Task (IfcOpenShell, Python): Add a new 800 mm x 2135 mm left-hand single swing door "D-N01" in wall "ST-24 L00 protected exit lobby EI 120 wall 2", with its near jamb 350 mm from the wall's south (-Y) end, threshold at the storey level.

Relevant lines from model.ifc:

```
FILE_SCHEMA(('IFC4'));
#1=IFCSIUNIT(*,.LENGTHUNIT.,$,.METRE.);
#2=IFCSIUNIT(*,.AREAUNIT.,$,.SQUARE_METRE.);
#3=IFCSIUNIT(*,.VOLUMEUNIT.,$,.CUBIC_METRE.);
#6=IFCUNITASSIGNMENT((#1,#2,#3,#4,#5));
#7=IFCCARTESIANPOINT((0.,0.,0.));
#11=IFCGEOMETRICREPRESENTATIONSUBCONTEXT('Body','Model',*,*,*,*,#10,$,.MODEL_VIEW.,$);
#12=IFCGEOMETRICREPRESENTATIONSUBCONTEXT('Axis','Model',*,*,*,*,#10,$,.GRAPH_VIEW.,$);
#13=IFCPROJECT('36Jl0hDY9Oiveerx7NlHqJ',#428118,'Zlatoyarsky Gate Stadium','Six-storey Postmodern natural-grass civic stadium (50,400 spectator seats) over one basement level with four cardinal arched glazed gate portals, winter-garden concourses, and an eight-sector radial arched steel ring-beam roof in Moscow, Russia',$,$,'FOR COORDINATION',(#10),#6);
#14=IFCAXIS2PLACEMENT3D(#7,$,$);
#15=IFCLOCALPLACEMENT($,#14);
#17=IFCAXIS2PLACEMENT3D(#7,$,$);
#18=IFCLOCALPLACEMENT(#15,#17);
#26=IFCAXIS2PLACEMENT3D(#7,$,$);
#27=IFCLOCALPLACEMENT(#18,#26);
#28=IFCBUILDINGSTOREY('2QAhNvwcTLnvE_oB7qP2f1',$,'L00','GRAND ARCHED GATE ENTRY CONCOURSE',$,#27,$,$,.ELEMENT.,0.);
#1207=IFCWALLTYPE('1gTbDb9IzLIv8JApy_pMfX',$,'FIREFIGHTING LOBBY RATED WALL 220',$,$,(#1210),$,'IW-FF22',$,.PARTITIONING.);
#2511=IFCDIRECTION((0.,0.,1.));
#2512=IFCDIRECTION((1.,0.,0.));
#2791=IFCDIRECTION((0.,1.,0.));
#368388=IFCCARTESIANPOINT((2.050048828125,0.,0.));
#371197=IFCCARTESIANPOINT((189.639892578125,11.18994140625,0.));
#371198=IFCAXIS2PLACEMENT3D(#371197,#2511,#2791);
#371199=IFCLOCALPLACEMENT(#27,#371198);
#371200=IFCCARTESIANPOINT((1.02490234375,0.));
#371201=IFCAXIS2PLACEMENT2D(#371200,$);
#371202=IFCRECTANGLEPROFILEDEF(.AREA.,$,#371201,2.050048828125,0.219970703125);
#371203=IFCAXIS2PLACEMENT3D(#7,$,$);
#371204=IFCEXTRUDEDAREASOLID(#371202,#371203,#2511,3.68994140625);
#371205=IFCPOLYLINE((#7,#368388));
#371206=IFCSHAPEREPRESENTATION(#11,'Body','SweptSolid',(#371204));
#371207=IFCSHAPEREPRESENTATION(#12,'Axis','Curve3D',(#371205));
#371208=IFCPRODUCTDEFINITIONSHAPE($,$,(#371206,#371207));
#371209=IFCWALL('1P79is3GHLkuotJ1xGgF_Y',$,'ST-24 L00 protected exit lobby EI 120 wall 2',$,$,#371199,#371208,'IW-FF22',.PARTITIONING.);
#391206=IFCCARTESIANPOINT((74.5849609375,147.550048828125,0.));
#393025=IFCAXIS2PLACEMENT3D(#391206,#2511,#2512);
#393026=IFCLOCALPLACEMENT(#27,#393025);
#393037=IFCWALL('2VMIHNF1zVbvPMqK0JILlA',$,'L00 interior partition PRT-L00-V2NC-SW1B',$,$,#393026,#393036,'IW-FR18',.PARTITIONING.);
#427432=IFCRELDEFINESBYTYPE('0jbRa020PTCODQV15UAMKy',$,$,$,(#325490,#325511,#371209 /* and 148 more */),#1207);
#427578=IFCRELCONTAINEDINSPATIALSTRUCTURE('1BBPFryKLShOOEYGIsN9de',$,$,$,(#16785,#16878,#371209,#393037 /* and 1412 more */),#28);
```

```python
import numpy as np
import ifcopenshell
import ifcopenshell.api.feature
import ifcopenshell.api.geometry
import ifcopenshell.api.root
import ifcopenshell.api.spatial
import ifcopenshell.geom
import ifcopenshell.util.element
import ifcopenshell.util.placement
import ifcopenshell.util.representation
import ifcopenshell.util.shape
import ifcopenshell.util.unit

model = ifcopenshell.open("model.ifc")
unit_scale = ifcopenshell.util.unit.calculate_unit_scale(model)
settings = ifcopenshell.geom.settings()


def volume(element):
    """Net volume in cubic metres, openings subtracted."""
    shape = ifcopenshell.geom.create_shape(settings, element)
    return ifcopenshell.util.shape.get_volume(shape.geometry)


wall = model.by_id(371209)
storey = ifcopenshell.util.element.get_container(wall, ifc_class="IfcBuildingStorey")
context = ifcopenshell.util.representation.get_context(model, "Model", "Body", "MODEL_VIEW")
before = volume(wall)

width, height, from_end, sill = 0.8, 2.135, 0.35, 0.0  # metres

# The wall runs along its own X axis, and the end named is its -X end.
wall_shape = ifcopenshell.geom.create_shape(settings, wall)
x, y, z = ifcopenshell.util.shape.get_vertices(wall_shape.geometry).T
start = x.min() + from_end
face, thickness = float(y.min()), float(y.max() - y.min())
wall_matrix = ifcopenshell.util.placement.get_local_placement(wall.ObjectPlacement)
level = ifcopenshell.util.placement.get_local_placement(storey.ObjectPlacement)[2, 3]


def in_wall(x, y):
    """Placement at x, y metres in the wall's axes, at sill height."""
    matrix = wall_matrix.copy()
    matrix[:, 3] = wall_matrix @ np.array([x / unit_scale, y / unit_scale, 0.0, 1.0])
    matrix[2, 3] = level + sill / unit_scale
    return matrix


# Opening: a box that overshoots both wall faces by 50 mm.
opening = ifcopenshell.api.root.create_entity(model, ifc_class="IfcOpeningElement", predefined_type="OPENING")
box = ifcopenshell.api.geometry.add_wall_representation(
    model, context=context, length=width, height=height, thickness=thickness + 0.1
)
ifcopenshell.api.geometry.assign_representation(model, product=opening, representation=box)
ifcopenshell.api.geometry.edit_object_placement(model, product=opening, matrix=in_wall(start, face - 0.05), is_si=False)
ifcopenshell.api.feature.add_feature(model, feature=opening, element=wall)

door = ifcopenshell.api.root.create_entity(model, ifc_class="IfcDoor", name="D-N01", predefined_type="DOOR")
door.OverallWidth, door.OverallHeight = width / unit_scale, height / unit_scale
door.OperationType = "SINGLE_SWING_LEFT"
body = ifcopenshell.api.geometry.add_door_representation(
    model,
    context=context,
    overall_width=door.OverallWidth,
    overall_height=door.OverallHeight,
    operation_type="SINGLE_SWING_LEFT",
    lining_properties={"LiningDepth": thickness / unit_scale, "ThresholdDepth": thickness / unit_scale},
)
ifcopenshell.api.geometry.assign_representation(model, product=door, representation=body)
ifcopenshell.api.spatial.assign_container(model, products=[door], relating_structure=storey)
ifcopenshell.api.feature.add_filling(model, opening=opening, element=door)

# The lining spans the wall, so the door starts at the wall face.
ifcopenshell.api.geometry.edit_object_placement(model, product=door, matrix=in_wall(start, face), is_si=False)

after = volume(wall)

print(f"wall volume {before:.3f} -> {after:.3f} m3")

model.write("model_edited.ifc")
```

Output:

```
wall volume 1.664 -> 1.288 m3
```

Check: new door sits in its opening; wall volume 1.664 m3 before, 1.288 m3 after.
